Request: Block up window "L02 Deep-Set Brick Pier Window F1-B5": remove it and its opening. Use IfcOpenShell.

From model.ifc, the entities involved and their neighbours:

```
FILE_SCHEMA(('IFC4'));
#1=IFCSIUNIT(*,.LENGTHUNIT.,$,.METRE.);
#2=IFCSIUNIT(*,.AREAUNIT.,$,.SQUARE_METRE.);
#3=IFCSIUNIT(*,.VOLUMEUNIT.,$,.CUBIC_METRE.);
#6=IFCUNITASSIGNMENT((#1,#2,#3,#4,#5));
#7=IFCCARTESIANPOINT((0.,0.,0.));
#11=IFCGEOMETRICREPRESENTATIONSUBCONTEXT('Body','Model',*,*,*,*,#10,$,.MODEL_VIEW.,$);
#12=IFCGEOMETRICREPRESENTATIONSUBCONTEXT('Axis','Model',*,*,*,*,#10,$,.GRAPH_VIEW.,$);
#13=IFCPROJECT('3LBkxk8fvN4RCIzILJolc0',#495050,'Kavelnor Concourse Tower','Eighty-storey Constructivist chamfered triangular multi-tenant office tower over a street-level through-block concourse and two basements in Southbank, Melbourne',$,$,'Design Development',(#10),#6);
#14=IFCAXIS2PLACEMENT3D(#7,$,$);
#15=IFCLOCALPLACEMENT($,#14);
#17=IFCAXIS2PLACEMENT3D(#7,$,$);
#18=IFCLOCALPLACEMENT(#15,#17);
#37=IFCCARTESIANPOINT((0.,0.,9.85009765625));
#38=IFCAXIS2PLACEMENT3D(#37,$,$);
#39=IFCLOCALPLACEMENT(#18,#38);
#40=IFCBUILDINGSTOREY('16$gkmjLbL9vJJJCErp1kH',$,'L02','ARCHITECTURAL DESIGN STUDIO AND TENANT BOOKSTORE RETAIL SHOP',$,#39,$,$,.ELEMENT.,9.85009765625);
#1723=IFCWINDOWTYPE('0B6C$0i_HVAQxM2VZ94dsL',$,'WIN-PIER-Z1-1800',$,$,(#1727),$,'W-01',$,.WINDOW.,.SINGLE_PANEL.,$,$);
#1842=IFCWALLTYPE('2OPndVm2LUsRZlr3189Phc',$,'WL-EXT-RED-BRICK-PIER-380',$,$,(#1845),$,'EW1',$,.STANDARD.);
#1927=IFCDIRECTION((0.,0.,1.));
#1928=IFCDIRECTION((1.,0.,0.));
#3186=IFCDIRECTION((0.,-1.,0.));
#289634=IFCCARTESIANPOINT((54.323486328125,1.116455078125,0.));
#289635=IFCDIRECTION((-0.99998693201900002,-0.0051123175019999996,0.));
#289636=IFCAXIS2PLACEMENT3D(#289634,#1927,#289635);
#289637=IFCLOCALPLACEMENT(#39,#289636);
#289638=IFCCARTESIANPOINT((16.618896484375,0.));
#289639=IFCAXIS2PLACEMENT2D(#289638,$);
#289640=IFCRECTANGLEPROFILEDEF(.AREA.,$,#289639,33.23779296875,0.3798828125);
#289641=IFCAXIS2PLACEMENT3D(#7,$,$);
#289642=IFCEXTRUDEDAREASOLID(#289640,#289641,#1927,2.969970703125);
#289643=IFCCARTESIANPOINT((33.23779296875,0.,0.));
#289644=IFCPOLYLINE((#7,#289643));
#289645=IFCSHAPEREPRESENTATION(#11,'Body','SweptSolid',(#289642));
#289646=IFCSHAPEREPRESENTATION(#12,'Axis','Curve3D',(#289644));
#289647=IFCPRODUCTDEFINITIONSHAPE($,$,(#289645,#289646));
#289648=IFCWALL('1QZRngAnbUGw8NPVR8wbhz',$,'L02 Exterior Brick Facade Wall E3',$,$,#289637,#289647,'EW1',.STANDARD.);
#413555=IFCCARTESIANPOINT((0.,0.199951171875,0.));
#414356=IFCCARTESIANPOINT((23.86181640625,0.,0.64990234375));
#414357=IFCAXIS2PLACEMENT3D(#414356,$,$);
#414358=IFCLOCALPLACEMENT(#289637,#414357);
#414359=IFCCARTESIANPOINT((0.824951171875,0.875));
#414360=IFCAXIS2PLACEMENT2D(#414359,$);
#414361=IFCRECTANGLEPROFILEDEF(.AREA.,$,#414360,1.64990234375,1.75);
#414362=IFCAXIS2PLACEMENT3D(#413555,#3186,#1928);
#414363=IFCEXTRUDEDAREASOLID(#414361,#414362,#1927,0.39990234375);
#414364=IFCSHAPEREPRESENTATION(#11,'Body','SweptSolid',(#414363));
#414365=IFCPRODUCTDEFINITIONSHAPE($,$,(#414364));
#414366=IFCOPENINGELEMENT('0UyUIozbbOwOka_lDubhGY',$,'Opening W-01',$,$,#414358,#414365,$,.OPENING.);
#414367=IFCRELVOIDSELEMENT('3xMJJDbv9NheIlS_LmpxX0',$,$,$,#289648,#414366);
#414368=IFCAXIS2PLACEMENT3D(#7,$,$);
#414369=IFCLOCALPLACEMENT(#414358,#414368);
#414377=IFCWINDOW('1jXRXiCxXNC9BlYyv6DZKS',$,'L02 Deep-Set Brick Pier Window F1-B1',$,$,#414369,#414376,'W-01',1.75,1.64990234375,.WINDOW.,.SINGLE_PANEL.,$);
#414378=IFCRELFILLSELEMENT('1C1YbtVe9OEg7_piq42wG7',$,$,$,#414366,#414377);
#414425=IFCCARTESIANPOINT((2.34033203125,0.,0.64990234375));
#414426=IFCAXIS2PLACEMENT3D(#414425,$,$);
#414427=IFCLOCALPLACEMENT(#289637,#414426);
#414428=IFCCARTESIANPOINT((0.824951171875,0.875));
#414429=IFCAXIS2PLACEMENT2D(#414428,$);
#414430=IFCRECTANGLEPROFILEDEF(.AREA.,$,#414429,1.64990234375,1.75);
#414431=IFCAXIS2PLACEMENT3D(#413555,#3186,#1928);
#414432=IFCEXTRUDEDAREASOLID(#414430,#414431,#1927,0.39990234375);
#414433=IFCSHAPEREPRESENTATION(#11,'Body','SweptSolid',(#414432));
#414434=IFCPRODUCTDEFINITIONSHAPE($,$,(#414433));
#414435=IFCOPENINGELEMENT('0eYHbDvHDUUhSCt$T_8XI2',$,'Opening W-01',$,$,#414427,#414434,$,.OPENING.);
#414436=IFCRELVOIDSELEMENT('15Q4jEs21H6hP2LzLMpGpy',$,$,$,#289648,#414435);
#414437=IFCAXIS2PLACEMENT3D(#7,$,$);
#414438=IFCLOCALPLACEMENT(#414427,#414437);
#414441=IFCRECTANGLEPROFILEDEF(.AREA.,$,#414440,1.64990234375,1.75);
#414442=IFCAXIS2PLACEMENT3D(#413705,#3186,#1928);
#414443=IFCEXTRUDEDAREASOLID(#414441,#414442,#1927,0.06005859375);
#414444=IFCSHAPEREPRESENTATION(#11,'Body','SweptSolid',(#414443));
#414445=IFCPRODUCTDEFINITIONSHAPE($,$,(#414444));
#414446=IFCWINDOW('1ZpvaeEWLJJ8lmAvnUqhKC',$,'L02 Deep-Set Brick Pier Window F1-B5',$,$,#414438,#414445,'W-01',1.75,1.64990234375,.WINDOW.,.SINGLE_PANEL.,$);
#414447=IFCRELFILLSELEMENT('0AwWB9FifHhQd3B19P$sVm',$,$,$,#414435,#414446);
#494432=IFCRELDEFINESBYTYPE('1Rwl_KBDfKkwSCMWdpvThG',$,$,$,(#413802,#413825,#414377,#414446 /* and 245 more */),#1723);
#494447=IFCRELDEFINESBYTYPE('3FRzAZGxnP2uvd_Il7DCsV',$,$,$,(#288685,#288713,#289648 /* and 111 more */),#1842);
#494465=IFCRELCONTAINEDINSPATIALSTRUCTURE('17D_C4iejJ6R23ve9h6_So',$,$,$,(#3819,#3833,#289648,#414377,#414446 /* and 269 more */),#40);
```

```python
import ifcopenshell
import ifcopenshell.api.feature
import ifcopenshell.api.root
import ifcopenshell.geom
import ifcopenshell.util.shape

model = ifcopenshell.open("model.ifc")
settings = ifcopenshell.geom.settings()


def volume(element):
    """Net volume in cubic metres, openings subtracted."""
    shape = ifcopenshell.geom.create_shape(settings, element)
    return ifcopenshell.util.shape.get_volume(shape.geometry)


window = model.by_guid("1ZpvaeEWLJJ8lmAvnUqhKC")
opening = window.FillsVoids[0].RelatingOpeningElement
wall = opening.VoidsElements[0].RelatingBuildingElement
before = volume(wall)

ifcopenshell.api.root.remove_product(model, product=window)
ifcopenshell.api.feature.remove_feature(model, feature=opening)

after = volume(wall)

print(f"wall volume {before:.3f} -> {after:.3f} m3")

model.write("model-out.ifc")
```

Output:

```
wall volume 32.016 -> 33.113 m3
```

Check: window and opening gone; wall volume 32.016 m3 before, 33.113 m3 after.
